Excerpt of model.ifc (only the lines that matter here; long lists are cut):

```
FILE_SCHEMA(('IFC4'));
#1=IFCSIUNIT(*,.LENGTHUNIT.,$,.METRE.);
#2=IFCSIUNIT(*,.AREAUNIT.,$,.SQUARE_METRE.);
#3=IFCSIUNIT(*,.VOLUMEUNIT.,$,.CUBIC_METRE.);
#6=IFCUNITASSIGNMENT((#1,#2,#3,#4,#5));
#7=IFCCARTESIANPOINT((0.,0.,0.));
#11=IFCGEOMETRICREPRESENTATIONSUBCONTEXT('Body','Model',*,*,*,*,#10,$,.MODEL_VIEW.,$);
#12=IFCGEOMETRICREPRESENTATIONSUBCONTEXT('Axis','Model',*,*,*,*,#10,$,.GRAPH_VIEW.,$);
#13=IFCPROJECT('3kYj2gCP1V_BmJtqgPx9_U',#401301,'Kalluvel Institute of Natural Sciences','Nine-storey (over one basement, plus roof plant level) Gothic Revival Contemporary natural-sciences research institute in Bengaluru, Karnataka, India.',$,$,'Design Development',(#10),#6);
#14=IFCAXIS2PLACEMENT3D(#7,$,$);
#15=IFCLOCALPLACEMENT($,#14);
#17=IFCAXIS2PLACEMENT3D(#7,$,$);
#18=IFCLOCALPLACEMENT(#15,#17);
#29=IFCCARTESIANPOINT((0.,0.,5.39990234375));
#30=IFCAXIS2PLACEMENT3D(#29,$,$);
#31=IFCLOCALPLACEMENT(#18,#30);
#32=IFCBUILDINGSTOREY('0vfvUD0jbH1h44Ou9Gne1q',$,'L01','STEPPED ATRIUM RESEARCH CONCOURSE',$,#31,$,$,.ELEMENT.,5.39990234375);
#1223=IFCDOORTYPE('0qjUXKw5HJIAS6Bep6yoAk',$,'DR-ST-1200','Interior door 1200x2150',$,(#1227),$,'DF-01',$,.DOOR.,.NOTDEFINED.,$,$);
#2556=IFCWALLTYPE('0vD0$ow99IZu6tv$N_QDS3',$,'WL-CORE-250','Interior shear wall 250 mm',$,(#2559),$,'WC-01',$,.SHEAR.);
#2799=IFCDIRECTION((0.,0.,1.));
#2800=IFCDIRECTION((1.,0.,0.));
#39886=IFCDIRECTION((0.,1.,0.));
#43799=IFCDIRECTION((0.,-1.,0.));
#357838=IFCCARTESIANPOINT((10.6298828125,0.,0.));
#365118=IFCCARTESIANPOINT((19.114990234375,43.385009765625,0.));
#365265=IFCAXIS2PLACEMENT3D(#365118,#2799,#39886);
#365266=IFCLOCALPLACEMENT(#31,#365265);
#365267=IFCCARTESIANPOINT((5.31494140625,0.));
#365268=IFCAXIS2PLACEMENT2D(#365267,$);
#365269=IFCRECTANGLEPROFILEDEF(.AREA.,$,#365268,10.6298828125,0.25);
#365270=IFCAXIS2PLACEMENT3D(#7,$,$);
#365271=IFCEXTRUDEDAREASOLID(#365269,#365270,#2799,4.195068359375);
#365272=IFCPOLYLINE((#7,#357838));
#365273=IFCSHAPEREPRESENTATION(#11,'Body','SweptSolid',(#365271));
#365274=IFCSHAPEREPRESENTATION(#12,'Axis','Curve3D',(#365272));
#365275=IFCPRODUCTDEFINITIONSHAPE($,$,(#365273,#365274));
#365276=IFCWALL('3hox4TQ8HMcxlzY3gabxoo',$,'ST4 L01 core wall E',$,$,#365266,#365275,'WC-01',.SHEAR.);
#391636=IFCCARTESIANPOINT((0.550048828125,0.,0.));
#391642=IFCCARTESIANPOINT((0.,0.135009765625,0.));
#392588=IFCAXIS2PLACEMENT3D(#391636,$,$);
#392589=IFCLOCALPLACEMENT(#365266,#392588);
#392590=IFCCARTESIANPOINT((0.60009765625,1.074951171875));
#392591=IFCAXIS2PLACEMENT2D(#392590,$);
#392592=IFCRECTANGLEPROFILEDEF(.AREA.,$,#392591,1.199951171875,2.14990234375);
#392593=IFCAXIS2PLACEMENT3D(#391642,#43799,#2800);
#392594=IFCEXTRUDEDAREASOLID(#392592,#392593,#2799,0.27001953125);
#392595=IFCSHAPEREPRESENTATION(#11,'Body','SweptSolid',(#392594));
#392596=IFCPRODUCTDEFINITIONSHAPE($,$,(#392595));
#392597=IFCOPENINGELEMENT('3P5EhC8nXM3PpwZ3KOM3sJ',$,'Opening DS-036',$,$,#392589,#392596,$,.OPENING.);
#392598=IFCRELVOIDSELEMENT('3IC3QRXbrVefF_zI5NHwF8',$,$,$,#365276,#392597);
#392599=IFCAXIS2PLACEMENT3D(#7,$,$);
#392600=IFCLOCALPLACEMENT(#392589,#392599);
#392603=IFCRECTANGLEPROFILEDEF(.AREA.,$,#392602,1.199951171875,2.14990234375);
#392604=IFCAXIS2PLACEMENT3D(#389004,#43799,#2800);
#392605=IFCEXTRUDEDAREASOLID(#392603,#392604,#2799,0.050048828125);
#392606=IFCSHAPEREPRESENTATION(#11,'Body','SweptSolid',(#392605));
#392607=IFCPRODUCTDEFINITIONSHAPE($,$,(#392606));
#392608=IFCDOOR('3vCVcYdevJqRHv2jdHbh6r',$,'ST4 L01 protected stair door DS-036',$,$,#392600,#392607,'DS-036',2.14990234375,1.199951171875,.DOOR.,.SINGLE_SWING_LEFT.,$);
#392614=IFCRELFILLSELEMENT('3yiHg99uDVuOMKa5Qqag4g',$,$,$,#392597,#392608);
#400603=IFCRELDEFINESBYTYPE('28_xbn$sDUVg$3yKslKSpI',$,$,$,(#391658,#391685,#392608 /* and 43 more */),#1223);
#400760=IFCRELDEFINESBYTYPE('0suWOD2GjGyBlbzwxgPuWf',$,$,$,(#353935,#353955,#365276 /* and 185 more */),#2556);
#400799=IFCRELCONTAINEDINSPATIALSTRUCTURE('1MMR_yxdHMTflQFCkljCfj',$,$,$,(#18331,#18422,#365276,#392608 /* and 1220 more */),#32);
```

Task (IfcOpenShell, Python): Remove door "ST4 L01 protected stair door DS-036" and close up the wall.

```python
import ifcopenshell
import ifcopenshell.api.feature
import ifcopenshell.api.root
import ifcopenshell.geom
import ifcopenshell.util.shape

model = ifcopenshell.open("model.ifc")
settings = ifcopenshell.geom.settings()


def volume(element):
    """Net volume in cubic metres, openings subtracted."""
    shape = ifcopenshell.geom.create_shape(settings, element)
    return ifcopenshell.util.shape.get_volume(shape.geometry)


door = model.by_guid("3vCVcYdevJqRHv2jdHbh6r")
opening = door.FillsVoids[0].RelatingOpeningElement
wall = opening.VoidsElements[0].RelatingBuildingElement
before = volume(wall)

ifcopenshell.api.root.remove_product(model, product=door)
ifcopenshell.api.feature.remove_feature(model, feature=opening)

after = volume(wall)

print(f"wall volume {before:.3f} -> {after:.3f} m3")

model.write("model_edited.ifc")
```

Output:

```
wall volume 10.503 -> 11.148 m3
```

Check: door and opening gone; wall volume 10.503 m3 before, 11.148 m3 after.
